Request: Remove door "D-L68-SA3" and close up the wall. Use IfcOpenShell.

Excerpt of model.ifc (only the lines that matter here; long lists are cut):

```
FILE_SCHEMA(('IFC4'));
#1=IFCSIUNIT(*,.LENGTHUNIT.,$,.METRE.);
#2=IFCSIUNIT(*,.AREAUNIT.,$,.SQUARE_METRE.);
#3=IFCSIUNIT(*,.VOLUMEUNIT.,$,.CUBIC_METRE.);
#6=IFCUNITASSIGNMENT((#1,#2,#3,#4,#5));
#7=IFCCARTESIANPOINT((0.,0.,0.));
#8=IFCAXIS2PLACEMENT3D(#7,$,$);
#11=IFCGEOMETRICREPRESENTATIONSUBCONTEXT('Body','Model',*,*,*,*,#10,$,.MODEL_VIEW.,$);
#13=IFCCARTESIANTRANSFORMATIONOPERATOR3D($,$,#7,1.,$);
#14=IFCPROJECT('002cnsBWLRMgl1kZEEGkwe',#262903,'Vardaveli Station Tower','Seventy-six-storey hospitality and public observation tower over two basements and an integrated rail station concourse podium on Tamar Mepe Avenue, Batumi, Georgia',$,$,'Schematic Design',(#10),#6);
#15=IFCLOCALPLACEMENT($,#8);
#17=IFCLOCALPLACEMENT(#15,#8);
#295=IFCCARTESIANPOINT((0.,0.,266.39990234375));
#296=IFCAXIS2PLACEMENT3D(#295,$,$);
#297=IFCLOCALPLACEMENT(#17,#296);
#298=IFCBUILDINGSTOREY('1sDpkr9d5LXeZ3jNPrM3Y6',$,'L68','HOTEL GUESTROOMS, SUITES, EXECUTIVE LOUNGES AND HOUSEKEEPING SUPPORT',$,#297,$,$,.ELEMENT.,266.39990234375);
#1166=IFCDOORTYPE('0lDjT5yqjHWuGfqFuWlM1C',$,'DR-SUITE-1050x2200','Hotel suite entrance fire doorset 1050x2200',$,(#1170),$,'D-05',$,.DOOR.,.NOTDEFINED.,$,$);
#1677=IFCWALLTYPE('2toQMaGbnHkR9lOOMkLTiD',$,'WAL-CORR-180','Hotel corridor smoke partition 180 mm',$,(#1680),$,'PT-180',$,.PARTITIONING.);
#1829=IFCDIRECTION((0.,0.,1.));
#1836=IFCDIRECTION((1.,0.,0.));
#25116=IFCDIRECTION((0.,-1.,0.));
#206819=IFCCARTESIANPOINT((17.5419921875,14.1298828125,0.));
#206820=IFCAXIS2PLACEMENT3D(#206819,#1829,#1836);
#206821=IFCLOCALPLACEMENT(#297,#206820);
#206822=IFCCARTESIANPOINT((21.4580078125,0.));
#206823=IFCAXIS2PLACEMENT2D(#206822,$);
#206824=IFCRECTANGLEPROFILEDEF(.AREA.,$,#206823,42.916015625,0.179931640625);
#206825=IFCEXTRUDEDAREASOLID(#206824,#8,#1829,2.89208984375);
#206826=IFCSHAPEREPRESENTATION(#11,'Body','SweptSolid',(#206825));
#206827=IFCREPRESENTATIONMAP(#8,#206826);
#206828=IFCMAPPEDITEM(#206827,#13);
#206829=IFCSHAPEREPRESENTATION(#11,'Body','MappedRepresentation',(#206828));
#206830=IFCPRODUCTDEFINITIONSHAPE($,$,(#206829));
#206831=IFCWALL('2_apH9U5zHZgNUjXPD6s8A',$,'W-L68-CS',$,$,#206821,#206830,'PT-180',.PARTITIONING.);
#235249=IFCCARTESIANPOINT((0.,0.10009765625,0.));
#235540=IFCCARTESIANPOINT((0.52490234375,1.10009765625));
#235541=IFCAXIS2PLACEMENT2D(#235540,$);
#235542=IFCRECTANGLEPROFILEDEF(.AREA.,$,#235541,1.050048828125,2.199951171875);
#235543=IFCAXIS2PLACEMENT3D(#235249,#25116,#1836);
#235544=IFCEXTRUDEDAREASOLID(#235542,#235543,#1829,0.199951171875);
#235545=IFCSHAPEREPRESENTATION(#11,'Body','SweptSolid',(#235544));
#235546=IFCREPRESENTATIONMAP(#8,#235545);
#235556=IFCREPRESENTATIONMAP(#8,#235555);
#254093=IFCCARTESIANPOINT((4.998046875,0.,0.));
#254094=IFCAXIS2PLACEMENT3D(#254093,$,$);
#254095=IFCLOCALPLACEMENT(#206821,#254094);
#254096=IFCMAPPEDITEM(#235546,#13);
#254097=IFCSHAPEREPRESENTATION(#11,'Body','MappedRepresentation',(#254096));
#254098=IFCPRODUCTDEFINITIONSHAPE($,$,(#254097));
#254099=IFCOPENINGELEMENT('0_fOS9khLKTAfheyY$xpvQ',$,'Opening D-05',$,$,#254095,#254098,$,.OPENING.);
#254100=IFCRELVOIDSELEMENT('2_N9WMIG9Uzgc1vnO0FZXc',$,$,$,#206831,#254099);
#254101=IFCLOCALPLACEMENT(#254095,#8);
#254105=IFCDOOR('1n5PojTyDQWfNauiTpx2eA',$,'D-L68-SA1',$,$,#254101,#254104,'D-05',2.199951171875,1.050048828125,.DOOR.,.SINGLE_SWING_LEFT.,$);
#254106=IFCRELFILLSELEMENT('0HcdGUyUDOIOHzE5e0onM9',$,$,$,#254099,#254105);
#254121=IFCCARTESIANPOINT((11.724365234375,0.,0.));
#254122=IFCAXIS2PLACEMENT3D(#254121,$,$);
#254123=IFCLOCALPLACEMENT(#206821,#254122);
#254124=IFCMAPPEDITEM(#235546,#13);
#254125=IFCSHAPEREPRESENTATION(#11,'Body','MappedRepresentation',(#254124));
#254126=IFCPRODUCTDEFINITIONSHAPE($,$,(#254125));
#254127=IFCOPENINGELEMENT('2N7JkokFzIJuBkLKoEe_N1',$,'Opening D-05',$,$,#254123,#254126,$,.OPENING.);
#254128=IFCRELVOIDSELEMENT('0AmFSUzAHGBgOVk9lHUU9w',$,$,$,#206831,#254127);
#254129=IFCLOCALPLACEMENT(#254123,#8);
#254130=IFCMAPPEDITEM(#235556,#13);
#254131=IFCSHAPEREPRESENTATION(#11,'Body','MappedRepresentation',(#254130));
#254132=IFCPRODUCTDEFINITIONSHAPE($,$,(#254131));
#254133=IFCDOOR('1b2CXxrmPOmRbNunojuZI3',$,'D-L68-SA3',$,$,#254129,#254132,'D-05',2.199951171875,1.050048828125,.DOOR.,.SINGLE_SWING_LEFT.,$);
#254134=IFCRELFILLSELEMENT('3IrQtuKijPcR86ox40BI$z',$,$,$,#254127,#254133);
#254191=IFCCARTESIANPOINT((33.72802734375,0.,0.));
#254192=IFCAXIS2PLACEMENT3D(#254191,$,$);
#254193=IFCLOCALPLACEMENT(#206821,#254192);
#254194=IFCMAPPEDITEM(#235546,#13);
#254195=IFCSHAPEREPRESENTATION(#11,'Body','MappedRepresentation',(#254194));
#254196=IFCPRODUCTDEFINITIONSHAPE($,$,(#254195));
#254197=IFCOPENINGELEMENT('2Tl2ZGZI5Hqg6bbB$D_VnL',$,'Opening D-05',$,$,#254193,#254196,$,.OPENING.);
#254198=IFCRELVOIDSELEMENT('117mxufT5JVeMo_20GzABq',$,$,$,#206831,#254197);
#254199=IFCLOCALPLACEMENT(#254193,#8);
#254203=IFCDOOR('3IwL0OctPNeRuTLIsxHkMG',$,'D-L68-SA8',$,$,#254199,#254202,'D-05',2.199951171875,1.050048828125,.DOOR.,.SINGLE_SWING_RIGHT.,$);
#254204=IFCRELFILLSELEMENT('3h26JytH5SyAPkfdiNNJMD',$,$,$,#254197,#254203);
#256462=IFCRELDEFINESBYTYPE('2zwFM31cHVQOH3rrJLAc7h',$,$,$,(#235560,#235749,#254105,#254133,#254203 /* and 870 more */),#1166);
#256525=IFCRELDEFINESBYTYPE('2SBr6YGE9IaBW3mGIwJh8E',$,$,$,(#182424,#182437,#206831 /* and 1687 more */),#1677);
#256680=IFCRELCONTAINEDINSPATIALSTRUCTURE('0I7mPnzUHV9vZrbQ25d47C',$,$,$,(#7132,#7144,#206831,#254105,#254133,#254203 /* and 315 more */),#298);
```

```python
import ifcopenshell
import ifcopenshell.api.feature
import ifcopenshell.api.root
import ifcopenshell.geom
import ifcopenshell.util.shape

model = ifcopenshell.open("model.ifc")
settings = ifcopenshell.geom.settings()


def volume(element):
    """Net volume in cubic metres, openings subtracted."""
    shape = ifcopenshell.geom.create_shape(settings, element)
    return ifcopenshell.util.shape.get_volume(shape.geometry)


door = model.by_guid("1b2CXxrmPOmRbNunojuZI3")
opening = door.FillsVoids[0].RelatingOpeningElement
wall = opening.VoidsElements[0].RelatingBuildingElement
before = volume(wall)

ifcopenshell.api.root.remove_product(model, product=door)
ifcopenshell.api.feature.remove_feature(model, feature=opening)

after = volume(wall)

print(f"wall volume {before:.3f} -> {after:.3f} m3")

model.write("model_updated.ifc")
```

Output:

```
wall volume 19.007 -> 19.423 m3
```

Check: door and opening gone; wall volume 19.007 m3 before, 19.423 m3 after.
